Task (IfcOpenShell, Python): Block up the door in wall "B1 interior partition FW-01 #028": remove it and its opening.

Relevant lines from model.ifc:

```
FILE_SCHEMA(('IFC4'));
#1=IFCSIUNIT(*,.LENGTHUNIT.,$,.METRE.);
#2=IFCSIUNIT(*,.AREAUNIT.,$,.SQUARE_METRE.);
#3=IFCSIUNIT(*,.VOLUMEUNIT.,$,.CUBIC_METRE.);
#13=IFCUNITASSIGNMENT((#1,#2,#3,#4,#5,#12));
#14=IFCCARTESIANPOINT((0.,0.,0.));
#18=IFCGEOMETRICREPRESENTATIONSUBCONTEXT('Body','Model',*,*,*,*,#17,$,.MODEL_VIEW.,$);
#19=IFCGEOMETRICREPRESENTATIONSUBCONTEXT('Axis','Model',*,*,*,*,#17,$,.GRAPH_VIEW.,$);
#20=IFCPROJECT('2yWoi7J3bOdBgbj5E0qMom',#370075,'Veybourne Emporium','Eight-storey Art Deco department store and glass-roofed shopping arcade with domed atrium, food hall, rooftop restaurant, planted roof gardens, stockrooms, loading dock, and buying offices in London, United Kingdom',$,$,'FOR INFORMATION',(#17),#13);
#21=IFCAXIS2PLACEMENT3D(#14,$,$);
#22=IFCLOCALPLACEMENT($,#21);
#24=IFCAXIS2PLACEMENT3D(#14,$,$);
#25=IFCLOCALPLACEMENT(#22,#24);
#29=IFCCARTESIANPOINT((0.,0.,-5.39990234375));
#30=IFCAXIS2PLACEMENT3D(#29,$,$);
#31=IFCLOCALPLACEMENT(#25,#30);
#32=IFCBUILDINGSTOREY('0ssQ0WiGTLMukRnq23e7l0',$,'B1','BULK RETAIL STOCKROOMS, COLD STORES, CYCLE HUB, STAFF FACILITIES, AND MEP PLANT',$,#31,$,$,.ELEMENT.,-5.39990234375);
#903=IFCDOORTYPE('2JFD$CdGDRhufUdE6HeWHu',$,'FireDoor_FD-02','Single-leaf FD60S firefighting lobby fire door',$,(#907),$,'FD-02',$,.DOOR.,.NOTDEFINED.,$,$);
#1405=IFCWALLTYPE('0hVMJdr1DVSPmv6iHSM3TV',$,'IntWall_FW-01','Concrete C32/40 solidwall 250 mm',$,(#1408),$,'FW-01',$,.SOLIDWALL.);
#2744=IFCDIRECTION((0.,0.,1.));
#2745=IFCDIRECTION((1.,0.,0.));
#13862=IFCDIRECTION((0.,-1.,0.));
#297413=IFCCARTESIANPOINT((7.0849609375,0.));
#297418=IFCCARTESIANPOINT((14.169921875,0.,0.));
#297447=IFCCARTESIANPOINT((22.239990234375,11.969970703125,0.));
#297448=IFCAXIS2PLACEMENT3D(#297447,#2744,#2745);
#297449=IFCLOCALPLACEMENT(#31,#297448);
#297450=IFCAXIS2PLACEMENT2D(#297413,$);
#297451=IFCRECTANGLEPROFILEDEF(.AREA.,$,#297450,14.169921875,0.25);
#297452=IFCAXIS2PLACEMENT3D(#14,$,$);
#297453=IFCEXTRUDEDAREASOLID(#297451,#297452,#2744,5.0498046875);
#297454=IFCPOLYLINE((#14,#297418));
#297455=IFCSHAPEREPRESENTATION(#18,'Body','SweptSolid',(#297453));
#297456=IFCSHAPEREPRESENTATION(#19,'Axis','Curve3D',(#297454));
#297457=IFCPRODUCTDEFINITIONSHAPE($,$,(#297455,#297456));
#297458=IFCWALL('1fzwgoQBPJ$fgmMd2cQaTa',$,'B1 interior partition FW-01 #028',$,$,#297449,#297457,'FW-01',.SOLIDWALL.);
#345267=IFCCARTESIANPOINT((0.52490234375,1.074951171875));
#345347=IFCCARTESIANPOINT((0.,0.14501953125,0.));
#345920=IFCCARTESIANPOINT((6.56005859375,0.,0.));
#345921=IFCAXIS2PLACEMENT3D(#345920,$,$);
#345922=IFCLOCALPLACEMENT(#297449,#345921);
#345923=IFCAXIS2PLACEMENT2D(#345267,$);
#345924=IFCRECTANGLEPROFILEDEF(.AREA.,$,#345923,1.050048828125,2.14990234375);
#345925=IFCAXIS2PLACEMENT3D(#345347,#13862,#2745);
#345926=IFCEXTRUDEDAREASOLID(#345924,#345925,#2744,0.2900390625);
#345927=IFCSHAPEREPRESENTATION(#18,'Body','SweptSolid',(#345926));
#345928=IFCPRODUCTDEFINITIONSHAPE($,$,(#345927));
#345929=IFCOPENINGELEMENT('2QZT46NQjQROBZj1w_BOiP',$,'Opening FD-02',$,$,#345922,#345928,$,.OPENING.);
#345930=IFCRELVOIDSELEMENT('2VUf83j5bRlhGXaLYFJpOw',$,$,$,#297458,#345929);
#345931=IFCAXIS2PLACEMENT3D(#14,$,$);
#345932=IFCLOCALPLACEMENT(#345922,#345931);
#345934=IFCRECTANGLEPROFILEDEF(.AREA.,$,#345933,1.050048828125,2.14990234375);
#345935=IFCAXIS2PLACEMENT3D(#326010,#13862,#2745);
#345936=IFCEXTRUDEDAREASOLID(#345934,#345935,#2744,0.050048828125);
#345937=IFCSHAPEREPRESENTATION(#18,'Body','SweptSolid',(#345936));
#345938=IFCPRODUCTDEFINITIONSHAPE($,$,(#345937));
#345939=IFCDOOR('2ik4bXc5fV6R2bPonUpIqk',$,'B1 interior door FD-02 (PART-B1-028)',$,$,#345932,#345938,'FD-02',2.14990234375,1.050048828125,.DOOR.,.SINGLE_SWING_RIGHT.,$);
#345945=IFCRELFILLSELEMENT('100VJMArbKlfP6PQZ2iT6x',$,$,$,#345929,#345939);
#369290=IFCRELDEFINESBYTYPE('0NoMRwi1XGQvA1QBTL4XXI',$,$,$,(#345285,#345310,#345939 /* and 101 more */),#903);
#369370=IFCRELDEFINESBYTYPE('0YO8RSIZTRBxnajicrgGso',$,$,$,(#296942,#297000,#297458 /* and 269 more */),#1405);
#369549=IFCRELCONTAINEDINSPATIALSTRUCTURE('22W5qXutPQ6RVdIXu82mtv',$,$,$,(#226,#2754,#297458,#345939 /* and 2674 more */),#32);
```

```python
import ifcopenshell
import ifcopenshell.api.feature
import ifcopenshell.api.root
import ifcopenshell.geom
import ifcopenshell.util.shape

model = ifcopenshell.open("model.ifc")
settings = ifcopenshell.geom.settings()


def volume(element):
    """Net volume in cubic metres, openings subtracted."""
    shape = ifcopenshell.geom.create_shape(settings, element)
    return ifcopenshell.util.shape.get_volume(shape.geometry)


door = model.by_guid("2ik4bXc5fV6R2bPonUpIqk")
opening = door.FillsVoids[0].RelatingOpeningElement
wall = opening.VoidsElements[0].RelatingBuildingElement
before = volume(wall)

ifcopenshell.api.root.remove_product(model, product=door)
ifcopenshell.api.feature.remove_feature(model, feature=opening)

after = volume(wall)

print(f"wall volume {before:.3f} -> {after:.3f} m3")

model.write("model_updated.ifc")
```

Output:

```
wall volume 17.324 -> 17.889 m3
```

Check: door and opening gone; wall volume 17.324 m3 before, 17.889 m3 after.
